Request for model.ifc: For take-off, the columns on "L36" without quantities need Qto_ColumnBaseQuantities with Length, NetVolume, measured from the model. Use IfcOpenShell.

First a look at what the model holds.

```python
import ifcopenshell
import ifcopenshell.util.element
import ifcopenshell.util.unit

model = ifcopenshell.open("model.ifc")
print(model.schema)
for unit_type in ("LENGTHUNIT", "AREAUNIT", "VOLUMEUNIT"):
    print(unit_type, ifcopenshell.util.unit.calculate_unit_scale(model, unit_type))
storey = next(s for s in model.by_type("IfcBuildingStorey") if s.Name == "L36")
columns = [e for e in ifcopenshell.util.element.get_decomposition(storey) if e.is_a("IfcColumn")]
for e in sorted(columns, key=lambda e: e.id()):
    print(e.id(), e.is_a(), e.Name, list(ifcopenshell.util.element.get_psets(e, qtos_only=True)), sep=" | ")
```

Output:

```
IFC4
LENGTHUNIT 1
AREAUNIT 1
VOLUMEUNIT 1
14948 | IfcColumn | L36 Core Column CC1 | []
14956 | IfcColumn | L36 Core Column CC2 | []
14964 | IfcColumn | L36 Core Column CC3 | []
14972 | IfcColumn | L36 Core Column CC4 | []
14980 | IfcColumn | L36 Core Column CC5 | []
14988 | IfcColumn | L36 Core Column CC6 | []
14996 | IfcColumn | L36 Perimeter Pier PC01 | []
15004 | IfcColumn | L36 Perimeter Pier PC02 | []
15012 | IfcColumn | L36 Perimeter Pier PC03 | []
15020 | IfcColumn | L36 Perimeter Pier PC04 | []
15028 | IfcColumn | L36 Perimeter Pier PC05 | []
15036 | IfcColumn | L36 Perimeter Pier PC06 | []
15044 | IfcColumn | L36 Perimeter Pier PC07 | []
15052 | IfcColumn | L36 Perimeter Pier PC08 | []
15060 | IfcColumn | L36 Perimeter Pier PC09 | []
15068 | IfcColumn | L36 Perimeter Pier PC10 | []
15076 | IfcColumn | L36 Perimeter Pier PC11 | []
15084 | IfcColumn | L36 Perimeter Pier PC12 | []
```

```python
import ifcopenshell
import ifcopenshell.api.pset
import ifcopenshell.geom
import ifcopenshell.util.element
import ifcopenshell.util.shape
import ifcopenshell.util.unit

model = ifcopenshell.open("model.ifc")
unit_scale = ifcopenshell.util.unit.calculate_unit_scale(model)
volume_scale = ifcopenshell.util.unit.calculate_unit_scale(model, "VOLUMEUNIT")
settings = ifcopenshell.geom.settings()

storey = next(s for s in model.by_type("IfcBuildingStorey") if s.Name == "L36")
columns = [e for e in ifcopenshell.util.element.get_decomposition(storey) if e.is_a("IfcColumn")]

for e in sorted(columns, key=lambda e: e.id()):
    if ifcopenshell.util.element.get_psets(e, qtos_only=True, should_inherit=False):
        continue
    # Geometry comes back in metres, in the element's own axes.
    shape = ifcopenshell.geom.create_shape(settings, e)
    values = {
        "Length": ifcopenshell.util.shape.get_z(shape.geometry) / unit_scale,
        "NetVolume": ifcopenshell.util.shape.get_volume(shape.geometry) / volume_scale,
    }
    qto = ifcopenshell.api.pset.add_qto(model, product=e, name="Qto_ColumnBaseQuantities")
    ifcopenshell.api.pset.edit_qto(model, qto=qto, properties=values)
    print(e.id(), {k: round(v, 3) for k, v in values.items()})

model.write("model-out.ifc")
```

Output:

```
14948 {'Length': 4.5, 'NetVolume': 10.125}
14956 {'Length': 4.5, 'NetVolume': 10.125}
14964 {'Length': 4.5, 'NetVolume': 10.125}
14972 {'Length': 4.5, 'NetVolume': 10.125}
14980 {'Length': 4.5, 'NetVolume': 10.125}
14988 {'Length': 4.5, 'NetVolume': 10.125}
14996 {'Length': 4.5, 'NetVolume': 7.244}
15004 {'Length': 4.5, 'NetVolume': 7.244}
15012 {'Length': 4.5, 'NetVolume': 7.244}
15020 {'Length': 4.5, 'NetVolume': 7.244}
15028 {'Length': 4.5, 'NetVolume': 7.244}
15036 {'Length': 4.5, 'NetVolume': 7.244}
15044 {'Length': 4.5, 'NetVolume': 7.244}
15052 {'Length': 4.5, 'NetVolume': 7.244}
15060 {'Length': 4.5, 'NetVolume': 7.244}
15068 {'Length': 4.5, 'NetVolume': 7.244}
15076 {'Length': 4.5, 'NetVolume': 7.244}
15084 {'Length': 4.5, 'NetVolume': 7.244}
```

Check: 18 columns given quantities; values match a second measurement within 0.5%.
